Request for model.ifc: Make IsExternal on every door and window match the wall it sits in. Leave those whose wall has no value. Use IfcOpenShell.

First a look at what the model holds.

```python
import ifcopenshell
import ifcopenshell.util.element

model = ifcopenshell.open("model.ifc")
print(model.schema)
seen = {}
for e in model.by_type("IfcDoor") + model.by_type("IfcWindow"):
    if not e.FillsVoids:
        continue
    host = e.FillsVoids[0].RelatingOpeningElement.VoidsElements[0].RelatingBuildingElement
    own = ifcopenshell.util.element.get_pset(e, f"Pset_{e.is_a()[3:].removesuffix('StandardCase')}Common", "IsExternal")
    wall = ifcopenshell.util.element.get_pset(host, "Pset_WallCommon", "IsExternal")
    seen[e.is_a(), own, wall] = seen.get((e.is_a(), own, wall), 0) + 1
for (cls, own, wall), count in sorted(seen.items(), key=str):
    print(count, cls, "IsExternal:", own, "| host wall:", wall)
```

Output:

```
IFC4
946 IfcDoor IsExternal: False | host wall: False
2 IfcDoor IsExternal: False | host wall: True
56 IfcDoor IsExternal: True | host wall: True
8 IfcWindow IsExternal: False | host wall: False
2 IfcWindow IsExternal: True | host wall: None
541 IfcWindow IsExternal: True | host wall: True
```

```python
import ifcopenshell
import ifcopenshell.api.pset
import ifcopenshell.util.element

model = ifcopenshell.open("model.ifc")

count = 0
for ifc_class, pset_name in (("IfcDoor", "Pset_DoorCommon"), ("IfcWindow", "Pset_WindowCommon")):
    for e in model.by_type(ifc_class):
        if not e.FillsVoids:
            continue
        host = e.FillsVoids[0].RelatingOpeningElement.VoidsElements[0].RelatingBuildingElement
        external = ifcopenshell.util.element.get_pset(host, "Pset_WallCommon", "IsExternal")
        if external is None or ifcopenshell.util.element.get_pset(e, pset_name, "IsExternal") == external:
            continue
        pset = ifcopenshell.api.pset.add_pset(model, product=e, name=pset_name)
        ifcopenshell.api.pset.edit_pset(model, pset=pset, properties={"IsExternal": external})
        count += 1

print(count, "updated")

model.write("model_v2.ifc")
```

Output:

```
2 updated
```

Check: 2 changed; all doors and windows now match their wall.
